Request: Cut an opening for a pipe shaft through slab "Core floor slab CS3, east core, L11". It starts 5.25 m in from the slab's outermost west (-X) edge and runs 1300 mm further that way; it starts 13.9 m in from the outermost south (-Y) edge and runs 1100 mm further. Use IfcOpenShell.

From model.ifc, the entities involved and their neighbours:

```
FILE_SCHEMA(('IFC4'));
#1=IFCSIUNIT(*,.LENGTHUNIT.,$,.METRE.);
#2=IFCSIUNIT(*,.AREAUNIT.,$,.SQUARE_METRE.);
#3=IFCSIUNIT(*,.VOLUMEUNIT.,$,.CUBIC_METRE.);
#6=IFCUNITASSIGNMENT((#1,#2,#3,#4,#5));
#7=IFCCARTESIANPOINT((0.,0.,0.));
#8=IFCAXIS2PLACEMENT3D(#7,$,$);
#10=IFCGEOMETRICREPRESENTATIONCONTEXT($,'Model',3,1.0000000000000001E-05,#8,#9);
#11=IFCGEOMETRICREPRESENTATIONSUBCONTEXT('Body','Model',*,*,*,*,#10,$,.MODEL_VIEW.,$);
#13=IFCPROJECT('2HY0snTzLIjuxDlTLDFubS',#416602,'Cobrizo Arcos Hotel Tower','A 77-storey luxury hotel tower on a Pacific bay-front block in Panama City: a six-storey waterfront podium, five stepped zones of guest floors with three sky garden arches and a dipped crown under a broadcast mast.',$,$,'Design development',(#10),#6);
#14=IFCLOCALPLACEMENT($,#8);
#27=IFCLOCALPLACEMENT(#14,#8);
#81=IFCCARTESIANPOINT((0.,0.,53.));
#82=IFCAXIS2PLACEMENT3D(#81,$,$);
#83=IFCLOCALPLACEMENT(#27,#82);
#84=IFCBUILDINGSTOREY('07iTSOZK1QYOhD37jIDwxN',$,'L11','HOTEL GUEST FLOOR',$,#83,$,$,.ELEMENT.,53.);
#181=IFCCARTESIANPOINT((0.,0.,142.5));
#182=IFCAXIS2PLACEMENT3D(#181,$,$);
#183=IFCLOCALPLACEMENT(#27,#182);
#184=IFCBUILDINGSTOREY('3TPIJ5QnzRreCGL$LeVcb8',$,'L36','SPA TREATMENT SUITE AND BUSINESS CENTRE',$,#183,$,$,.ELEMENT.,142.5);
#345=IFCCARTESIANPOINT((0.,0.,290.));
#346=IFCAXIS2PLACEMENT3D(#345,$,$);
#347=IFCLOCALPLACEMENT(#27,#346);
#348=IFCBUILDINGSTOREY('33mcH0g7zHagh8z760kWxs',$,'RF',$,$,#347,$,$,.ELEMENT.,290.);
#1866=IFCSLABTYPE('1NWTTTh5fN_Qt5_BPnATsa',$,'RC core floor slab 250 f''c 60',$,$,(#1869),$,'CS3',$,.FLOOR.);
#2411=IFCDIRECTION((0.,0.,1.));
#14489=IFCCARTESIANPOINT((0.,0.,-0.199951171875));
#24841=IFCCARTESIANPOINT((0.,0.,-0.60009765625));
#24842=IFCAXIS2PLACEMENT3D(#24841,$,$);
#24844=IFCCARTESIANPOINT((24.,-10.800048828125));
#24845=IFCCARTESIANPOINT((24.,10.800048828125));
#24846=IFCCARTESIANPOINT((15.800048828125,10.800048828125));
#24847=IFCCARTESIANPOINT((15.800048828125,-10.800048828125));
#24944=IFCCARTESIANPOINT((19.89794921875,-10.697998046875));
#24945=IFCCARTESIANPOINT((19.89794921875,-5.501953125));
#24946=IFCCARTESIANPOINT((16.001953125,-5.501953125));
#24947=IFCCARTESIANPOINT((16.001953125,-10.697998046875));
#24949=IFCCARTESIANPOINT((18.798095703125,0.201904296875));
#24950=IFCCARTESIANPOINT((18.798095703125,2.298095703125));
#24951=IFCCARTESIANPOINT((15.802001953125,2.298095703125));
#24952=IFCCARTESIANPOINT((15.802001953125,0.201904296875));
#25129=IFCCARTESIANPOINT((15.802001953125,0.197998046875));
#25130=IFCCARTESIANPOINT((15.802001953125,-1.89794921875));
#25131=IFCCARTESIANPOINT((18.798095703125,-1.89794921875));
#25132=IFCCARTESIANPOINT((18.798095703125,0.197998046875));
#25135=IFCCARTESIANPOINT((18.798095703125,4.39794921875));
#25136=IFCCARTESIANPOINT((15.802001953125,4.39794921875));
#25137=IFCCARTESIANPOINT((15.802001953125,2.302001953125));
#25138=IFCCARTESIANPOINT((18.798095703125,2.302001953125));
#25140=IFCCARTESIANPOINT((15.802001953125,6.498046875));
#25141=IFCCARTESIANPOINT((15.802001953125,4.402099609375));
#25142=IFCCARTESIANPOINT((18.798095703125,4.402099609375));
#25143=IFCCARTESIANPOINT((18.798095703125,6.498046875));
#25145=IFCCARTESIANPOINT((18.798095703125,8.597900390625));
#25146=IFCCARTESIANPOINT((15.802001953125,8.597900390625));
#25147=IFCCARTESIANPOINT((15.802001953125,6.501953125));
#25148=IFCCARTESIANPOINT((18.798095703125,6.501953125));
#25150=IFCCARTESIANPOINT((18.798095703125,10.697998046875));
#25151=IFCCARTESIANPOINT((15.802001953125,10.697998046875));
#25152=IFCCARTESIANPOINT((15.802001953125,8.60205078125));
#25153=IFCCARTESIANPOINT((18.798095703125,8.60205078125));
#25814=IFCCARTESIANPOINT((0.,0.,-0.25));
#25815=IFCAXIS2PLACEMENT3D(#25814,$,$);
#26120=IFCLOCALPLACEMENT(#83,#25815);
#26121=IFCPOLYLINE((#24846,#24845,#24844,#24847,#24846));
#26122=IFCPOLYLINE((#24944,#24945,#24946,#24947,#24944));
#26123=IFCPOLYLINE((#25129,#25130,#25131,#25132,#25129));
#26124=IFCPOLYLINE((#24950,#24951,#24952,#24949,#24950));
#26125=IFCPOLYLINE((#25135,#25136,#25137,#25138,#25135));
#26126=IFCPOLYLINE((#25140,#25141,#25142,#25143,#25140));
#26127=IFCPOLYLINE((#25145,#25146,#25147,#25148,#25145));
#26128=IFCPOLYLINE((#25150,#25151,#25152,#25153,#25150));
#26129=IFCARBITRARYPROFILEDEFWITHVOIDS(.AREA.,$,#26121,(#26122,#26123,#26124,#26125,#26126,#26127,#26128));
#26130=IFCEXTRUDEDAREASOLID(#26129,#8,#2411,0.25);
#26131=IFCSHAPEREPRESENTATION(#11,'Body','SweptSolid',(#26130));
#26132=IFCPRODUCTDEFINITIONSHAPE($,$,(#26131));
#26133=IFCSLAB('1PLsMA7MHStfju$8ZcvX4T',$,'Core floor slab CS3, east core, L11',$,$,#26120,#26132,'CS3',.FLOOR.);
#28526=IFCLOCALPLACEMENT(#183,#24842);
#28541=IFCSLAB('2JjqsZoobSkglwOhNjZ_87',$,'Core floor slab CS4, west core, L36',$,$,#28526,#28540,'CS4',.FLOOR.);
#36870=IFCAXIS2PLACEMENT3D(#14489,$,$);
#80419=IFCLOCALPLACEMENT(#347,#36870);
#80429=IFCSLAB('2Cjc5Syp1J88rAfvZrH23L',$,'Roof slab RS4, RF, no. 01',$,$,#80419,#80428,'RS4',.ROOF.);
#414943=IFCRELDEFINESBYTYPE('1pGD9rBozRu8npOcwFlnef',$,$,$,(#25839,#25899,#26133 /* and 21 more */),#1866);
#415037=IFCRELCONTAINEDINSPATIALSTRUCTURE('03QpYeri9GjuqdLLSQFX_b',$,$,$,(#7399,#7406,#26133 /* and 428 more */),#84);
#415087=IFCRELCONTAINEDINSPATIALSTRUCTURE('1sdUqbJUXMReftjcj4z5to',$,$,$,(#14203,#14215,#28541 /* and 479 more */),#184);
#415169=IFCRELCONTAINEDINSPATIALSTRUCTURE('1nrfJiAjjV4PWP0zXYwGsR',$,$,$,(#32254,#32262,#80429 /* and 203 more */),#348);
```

```python
import numpy as np
import ifcopenshell
import ifcopenshell.api.feature
import ifcopenshell.api.geometry
import ifcopenshell.api.root
import ifcopenshell.geom
import ifcopenshell.util.placement
import ifcopenshell.util.representation
import ifcopenshell.util.shape
import ifcopenshell.util.unit

model = ifcopenshell.open("model.ifc")
unit_scale = ifcopenshell.util.unit.calculate_unit_scale(model)
settings = ifcopenshell.geom.settings()


def volume(element):
    """Net volume in cubic metres, openings subtracted."""
    shape = ifcopenshell.geom.create_shape(settings, element)
    return ifcopenshell.util.shape.get_volume(shape.geometry)


slab = model.by_id(26133)
before = volume(slab)

# Extent in the slab's own axes, in metres. The edges named are its -X and -Y sides.
slab_shape = ifcopenshell.geom.create_shape(settings, slab)
vertices = ifcopenshell.util.shape.get_vertices(slab_shape.geometry)
x_min, y_min, bottom = vertices.min(axis=0)
top = vertices[:, 2].max()

opening = ifcopenshell.api.root.create_entity(model, ifc_class="IfcOpeningElement", name="Pipe shaft opening", predefined_type="OPENING")
context = ifcopenshell.util.representation.get_context(model, "Model", "Body", "MODEL_VIEW")
width, depth = 1.3, 1.1
outline = [(0.0, 0.0), (width, 0.0), (width, depth), (0.0, depth), (0.0, 0.0)]
# Overshoot both faces by 50 mm so the cut is clean.
shape = ifcopenshell.api.geometry.add_slab_representation(
    model, context=context, depth=top - bottom + 0.1, polyline=outline
)
ifcopenshell.api.geometry.assign_representation(model, product=opening, representation=shape)

matrix = ifcopenshell.util.placement.get_local_placement(slab.ObjectPlacement)
matrix[:, 3] = matrix @ np.append(np.array([x_min + 5.25, y_min + 13.9, bottom - 0.05]) / unit_scale, 1.0)
ifcopenshell.api.geometry.edit_object_placement(model, product=opening, matrix=matrix, is_si=False)
ifcopenshell.api.feature.add_feature(model, feature=opening, element=slab)

after = volume(slab)

print(f"slab volume {before:.3f} -> {after:.3f} m3")

model.write("model_rev.ifc")
```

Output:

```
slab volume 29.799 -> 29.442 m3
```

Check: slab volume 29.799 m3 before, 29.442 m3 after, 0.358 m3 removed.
